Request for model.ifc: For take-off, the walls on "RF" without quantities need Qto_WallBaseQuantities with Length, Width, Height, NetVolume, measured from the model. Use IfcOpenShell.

First a look at what the model holds.

```python
import ifcopenshell
import ifcopenshell.util.element
import ifcopenshell.util.unit

model = ifcopenshell.open("model.ifc")
print(model.schema)
for unit_type in ("LENGTHUNIT", "AREAUNIT", "VOLUMEUNIT"):
    print(unit_type, ifcopenshell.util.unit.calculate_unit_scale(model, unit_type))
storey = next(s for s in model.by_type("IfcBuildingStorey") if s.Name == "RF")
walls = [e for e in ifcopenshell.util.element.get_decomposition(storey) if e.is_a("IfcWall")]
for e in sorted(walls, key=lambda e: e.id()):
    print(e.id(), e.is_a(), e.Name, list(ifcopenshell.util.element.get_psets(e, qtos_only=True)), sep=" | ")
```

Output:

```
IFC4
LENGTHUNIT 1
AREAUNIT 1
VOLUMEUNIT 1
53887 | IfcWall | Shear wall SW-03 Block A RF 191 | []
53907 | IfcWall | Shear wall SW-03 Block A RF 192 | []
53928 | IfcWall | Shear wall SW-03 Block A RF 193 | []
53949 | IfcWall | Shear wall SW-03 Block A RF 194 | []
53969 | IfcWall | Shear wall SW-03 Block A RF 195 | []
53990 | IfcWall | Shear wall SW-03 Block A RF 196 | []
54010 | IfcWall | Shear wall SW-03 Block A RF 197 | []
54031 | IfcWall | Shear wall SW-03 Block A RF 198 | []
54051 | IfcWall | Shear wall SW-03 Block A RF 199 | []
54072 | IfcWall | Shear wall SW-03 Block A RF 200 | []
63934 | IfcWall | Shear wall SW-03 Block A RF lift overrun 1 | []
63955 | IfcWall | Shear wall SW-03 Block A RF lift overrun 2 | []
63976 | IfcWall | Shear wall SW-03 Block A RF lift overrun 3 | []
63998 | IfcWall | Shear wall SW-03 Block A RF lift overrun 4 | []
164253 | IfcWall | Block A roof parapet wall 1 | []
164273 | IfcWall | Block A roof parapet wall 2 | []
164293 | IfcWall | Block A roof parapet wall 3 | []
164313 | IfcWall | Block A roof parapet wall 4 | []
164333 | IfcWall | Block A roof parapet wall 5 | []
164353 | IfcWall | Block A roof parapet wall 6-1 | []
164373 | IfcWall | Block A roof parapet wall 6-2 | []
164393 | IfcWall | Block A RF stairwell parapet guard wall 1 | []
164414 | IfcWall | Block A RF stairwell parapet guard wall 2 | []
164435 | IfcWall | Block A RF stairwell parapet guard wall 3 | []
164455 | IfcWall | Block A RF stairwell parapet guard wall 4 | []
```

```python
import ifcopenshell
import ifcopenshell.api.pset
import ifcopenshell.geom
import ifcopenshell.util.element
import ifcopenshell.util.shape
import ifcopenshell.util.unit

model = ifcopenshell.open("model.ifc")
unit_scale = ifcopenshell.util.unit.calculate_unit_scale(model)
volume_scale = ifcopenshell.util.unit.calculate_unit_scale(model, "VOLUMEUNIT")
settings = ifcopenshell.geom.settings()

storey = next(s for s in model.by_type("IfcBuildingStorey") if s.Name == "RF")
walls = [e for e in ifcopenshell.util.element.get_decomposition(storey) if e.is_a("IfcWall")]

for e in sorted(walls, key=lambda e: e.id()):
    if ifcopenshell.util.element.get_psets(e, qtos_only=True, should_inherit=False):
        continue
    # Geometry comes back in metres, in the element's own axes.
    shape = ifcopenshell.geom.create_shape(settings, e)
    values = {
        "Length": ifcopenshell.util.shape.get_x(shape.geometry) / unit_scale,
        "Width": ifcopenshell.util.shape.get_y(shape.geometry) / unit_scale,
        "Height": ifcopenshell.util.shape.get_z(shape.geometry) / unit_scale,
        "NetVolume": ifcopenshell.util.shape.get_volume(shape.geometry) / volume_scale,
    }
    qto = ifcopenshell.api.pset.add_qto(model, product=e, name="Qto_WallBaseQuantities")
    ifcopenshell.api.pset.edit_qto(model, qto=qto, properties=values)
    print(e.id(), {k: round(v, 3) for k, v in values.items()})

model.write("model-out.ifc")
```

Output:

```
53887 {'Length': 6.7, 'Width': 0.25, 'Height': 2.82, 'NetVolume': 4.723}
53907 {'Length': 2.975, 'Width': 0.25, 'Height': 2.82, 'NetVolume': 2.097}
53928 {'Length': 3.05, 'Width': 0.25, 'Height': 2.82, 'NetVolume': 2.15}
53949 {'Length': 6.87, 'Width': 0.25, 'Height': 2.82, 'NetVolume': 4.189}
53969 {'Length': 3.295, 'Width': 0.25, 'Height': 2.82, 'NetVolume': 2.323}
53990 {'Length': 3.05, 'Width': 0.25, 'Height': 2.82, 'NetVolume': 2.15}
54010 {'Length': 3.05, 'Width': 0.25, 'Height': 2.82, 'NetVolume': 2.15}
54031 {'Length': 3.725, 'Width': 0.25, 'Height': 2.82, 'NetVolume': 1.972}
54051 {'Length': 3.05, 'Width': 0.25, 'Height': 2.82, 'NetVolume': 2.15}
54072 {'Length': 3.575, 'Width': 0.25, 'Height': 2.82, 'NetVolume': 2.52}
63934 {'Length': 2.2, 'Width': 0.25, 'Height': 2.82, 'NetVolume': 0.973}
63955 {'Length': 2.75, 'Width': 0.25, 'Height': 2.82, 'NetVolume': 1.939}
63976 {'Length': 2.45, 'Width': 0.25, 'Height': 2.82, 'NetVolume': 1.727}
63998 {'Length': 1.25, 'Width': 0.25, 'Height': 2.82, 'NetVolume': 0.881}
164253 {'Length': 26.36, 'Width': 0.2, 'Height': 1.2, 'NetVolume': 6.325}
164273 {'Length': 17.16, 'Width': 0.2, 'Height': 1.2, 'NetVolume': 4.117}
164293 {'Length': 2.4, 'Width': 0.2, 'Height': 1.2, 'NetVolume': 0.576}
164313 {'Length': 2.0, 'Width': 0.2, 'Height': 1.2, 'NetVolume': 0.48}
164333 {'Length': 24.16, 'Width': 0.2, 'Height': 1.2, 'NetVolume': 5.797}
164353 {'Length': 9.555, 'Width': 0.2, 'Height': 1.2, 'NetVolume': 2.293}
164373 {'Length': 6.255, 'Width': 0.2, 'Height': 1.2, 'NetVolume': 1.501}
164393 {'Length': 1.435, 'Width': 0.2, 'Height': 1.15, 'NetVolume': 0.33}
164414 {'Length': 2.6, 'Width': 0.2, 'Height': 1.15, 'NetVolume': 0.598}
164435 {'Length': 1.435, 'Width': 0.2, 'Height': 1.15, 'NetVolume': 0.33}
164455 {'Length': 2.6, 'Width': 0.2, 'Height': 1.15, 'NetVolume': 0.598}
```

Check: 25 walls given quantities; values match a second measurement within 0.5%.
